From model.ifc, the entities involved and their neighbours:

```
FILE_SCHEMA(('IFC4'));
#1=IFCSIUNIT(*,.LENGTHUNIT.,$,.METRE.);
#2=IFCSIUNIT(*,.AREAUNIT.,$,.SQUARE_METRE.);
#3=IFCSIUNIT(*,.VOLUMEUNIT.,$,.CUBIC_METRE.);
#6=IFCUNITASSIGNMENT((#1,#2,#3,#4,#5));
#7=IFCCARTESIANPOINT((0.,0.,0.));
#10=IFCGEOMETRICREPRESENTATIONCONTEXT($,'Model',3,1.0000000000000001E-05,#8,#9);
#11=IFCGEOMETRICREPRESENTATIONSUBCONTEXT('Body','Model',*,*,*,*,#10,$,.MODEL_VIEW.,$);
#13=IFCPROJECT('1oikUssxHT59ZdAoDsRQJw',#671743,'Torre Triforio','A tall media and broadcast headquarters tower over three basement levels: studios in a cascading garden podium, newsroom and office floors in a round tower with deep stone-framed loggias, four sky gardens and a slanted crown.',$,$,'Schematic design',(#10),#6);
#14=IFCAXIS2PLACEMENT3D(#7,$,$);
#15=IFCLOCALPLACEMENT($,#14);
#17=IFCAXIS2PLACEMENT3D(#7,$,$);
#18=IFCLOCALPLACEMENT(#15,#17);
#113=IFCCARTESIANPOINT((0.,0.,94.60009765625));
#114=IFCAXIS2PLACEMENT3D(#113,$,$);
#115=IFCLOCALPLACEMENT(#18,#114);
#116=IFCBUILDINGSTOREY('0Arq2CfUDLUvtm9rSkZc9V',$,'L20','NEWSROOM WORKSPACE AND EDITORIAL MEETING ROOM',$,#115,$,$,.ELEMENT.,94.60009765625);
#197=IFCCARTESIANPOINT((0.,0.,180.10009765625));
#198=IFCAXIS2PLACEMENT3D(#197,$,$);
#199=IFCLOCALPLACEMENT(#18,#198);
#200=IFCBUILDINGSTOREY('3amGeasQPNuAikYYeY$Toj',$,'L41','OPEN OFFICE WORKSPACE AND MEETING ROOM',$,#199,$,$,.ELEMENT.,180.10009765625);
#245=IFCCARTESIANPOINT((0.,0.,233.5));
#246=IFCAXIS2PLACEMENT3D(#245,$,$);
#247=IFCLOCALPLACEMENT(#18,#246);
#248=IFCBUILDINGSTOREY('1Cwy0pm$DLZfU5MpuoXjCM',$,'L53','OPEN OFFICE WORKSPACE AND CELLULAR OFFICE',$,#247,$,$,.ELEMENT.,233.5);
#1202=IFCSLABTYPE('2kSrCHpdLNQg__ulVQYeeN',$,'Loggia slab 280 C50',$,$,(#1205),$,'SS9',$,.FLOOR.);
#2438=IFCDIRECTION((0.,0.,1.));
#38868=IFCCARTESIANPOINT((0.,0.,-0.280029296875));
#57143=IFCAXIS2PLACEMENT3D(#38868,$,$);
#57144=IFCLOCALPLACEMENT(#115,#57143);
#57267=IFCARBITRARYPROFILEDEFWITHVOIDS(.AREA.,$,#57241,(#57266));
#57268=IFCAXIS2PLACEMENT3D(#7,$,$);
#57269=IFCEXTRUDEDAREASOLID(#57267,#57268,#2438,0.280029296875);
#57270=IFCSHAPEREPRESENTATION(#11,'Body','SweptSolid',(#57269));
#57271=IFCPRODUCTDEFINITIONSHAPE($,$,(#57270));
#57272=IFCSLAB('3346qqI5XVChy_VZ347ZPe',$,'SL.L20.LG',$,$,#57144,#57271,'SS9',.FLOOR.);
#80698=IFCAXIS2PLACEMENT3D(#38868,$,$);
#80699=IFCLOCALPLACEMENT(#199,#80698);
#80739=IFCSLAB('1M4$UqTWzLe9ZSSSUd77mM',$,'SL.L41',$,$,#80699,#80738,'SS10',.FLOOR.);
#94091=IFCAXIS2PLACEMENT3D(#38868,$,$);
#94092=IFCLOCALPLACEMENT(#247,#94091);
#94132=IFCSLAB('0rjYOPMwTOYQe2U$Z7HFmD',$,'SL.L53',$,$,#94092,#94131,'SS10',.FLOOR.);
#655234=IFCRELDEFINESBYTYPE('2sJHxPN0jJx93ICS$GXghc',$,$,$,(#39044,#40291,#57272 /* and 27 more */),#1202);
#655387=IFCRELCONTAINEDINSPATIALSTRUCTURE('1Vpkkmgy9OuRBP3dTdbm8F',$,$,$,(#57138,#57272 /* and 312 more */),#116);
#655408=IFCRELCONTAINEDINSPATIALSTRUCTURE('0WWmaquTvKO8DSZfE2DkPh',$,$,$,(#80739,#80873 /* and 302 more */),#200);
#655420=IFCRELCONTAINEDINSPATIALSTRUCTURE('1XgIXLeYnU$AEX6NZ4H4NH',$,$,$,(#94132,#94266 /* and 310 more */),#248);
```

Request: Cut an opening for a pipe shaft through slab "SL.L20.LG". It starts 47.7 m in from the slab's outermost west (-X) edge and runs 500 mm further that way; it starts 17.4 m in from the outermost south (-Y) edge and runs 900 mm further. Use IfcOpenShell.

```python
import numpy as np
import ifcopenshell
import ifcopenshell.api.feature
import ifcopenshell.api.geometry
import ifcopenshell.api.root
import ifcopenshell.geom
import ifcopenshell.util.placement
import ifcopenshell.util.representation
import ifcopenshell.util.shape
import ifcopenshell.util.unit

model = ifcopenshell.open("model.ifc")
unit_scale = ifcopenshell.util.unit.calculate_unit_scale(model)
settings = ifcopenshell.geom.settings()


def volume(element):
    """Net volume in cubic metres, openings subtracted."""
    shape = ifcopenshell.geom.create_shape(settings, element)
    return ifcopenshell.util.shape.get_volume(shape.geometry)


slab = model.by_guid("3346qqI5XVChy_VZ347ZPe")
before = volume(slab)

# Extent in the slab's own axes, in metres. The edges named are its -X and -Y sides.
slab_shape = ifcopenshell.geom.create_shape(settings, slab)
vertices = ifcopenshell.util.shape.get_vertices(slab_shape.geometry)
x_min, y_min, bottom = vertices.min(axis=0)
top = vertices[:, 2].max()

opening = ifcopenshell.api.root.create_entity(model, ifc_class="IfcOpeningElement", name="Pipe shaft opening", predefined_type="OPENING")
context = ifcopenshell.util.representation.get_context(model, "Model", "Body", "MODEL_VIEW")
width, depth = 0.5, 0.9
outline = [(0.0, 0.0), (width, 0.0), (width, depth), (0.0, depth), (0.0, 0.0)]
# Overshoot both faces by 50 mm so the cut is clean.
shape = ifcopenshell.api.geometry.add_slab_representation(
    model, context=context, depth=top - bottom + 0.1, polyline=outline
)
ifcopenshell.api.geometry.assign_representation(model, product=opening, representation=shape)

matrix = ifcopenshell.util.placement.get_local_placement(slab.ObjectPlacement)
matrix[:, 3] = matrix @ np.append(np.array([x_min + 47.7, y_min + 17.4, bottom - 0.05]) / unit_scale, 1.0)
ifcopenshell.api.geometry.edit_object_placement(model, product=opening, matrix=matrix, is_si=False)
ifcopenshell.api.feature.add_feature(model, feature=opening, element=slab)

after = volume(slab)

print(f"slab volume {before:.3f} -> {after:.3f} m3")

model.write("model_edited.ifc")
```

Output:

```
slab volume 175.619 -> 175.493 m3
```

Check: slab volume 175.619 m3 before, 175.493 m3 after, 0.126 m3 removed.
